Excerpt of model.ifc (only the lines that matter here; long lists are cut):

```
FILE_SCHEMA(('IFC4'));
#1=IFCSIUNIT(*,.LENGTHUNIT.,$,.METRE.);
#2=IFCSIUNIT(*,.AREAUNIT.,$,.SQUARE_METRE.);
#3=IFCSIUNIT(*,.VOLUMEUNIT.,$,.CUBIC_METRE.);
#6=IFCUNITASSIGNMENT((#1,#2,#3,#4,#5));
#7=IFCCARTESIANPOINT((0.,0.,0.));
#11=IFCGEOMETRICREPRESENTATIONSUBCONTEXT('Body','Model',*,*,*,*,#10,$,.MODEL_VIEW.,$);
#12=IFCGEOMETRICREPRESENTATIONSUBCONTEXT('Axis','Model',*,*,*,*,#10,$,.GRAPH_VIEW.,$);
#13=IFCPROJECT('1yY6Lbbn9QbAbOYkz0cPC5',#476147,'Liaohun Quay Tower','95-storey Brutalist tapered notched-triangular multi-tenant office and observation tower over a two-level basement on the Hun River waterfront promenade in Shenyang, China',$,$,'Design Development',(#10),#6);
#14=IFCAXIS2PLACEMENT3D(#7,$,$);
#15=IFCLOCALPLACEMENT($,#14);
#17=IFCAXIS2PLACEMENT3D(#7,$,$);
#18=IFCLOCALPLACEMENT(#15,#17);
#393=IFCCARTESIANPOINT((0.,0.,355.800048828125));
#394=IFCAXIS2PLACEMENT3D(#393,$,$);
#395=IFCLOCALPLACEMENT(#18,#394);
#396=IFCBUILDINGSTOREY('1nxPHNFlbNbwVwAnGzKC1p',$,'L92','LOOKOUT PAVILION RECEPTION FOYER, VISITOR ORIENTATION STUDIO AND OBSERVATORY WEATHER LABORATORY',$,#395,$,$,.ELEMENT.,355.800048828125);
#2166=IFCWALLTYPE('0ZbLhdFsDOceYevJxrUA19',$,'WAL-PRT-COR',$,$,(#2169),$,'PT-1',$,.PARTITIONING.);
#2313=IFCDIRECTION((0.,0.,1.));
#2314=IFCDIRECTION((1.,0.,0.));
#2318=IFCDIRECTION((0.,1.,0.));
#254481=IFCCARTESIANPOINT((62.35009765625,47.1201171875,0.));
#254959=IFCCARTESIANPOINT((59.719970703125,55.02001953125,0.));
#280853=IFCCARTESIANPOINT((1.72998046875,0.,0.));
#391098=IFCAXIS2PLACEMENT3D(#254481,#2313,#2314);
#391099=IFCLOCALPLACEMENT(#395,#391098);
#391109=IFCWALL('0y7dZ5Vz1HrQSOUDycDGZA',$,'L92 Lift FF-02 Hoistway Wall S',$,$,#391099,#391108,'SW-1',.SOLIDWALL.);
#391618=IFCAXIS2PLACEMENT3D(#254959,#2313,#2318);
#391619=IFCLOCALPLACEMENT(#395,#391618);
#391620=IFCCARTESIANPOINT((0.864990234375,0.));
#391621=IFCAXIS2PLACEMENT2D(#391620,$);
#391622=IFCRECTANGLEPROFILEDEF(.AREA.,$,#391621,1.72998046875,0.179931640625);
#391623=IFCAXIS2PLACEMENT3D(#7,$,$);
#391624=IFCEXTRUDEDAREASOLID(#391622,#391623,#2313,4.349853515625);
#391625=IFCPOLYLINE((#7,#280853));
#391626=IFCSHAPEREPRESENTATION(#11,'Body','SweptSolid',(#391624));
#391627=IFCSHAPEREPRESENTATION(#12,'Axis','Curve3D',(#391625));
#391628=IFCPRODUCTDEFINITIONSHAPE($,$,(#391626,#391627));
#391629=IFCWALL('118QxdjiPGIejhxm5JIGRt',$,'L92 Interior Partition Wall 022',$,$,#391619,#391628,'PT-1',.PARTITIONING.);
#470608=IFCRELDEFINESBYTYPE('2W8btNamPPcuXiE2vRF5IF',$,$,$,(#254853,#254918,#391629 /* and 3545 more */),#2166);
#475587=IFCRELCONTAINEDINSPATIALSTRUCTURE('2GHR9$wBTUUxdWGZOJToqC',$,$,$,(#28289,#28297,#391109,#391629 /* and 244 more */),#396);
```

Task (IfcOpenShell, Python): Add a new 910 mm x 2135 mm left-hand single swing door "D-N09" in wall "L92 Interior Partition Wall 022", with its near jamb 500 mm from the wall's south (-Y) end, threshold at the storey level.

```python
import numpy as np
import ifcopenshell
import ifcopenshell.api.feature
import ifcopenshell.api.geometry
import ifcopenshell.api.root
import ifcopenshell.api.spatial
import ifcopenshell.geom
import ifcopenshell.util.element
import ifcopenshell.util.placement
import ifcopenshell.util.representation
import ifcopenshell.util.shape
import ifcopenshell.util.unit

model = ifcopenshell.open("model.ifc")
unit_scale = ifcopenshell.util.unit.calculate_unit_scale(model)
settings = ifcopenshell.geom.settings()


def volume(element):
    """Net volume in cubic metres, openings subtracted."""
    shape = ifcopenshell.geom.create_shape(settings, element)
    return ifcopenshell.util.shape.get_volume(shape.geometry)


wall = model.by_id(391629)
storey = ifcopenshell.util.element.get_container(wall, ifc_class="IfcBuildingStorey")
context = ifcopenshell.util.representation.get_context(model, "Model", "Body", "MODEL_VIEW")
before = volume(wall)

width, height, from_end, sill = 0.91, 2.135, 0.5, 0.0  # metres

# The wall runs along its own X axis, and the end named is its -X end.
wall_shape = ifcopenshell.geom.create_shape(settings, wall)
x, y, z = ifcopenshell.util.shape.get_vertices(wall_shape.geometry).T
start = x.min() + from_end
face, thickness = float(y.min()), float(y.max() - y.min())
wall_matrix = ifcopenshell.util.placement.get_local_placement(wall.ObjectPlacement)
level = ifcopenshell.util.placement.get_local_placement(storey.ObjectPlacement)[2, 3]


def in_wall(x, y):
    """Placement at x, y metres in the wall's axes, at sill height."""
    matrix = wall_matrix.copy()
    matrix[:, 3] = wall_matrix @ np.array([x / unit_scale, y / unit_scale, 0.0, 1.0])
    matrix[2, 3] = level + sill / unit_scale
    return matrix


# Opening: a box that overshoots both wall faces by 50 mm.
opening = ifcopenshell.api.root.create_entity(model, ifc_class="IfcOpeningElement", predefined_type="OPENING")
box = ifcopenshell.api.geometry.add_wall_representation(
    model, context=context, length=width, height=height, thickness=thickness + 0.1
)
ifcopenshell.api.geometry.assign_representation(model, product=opening, representation=box)
ifcopenshell.api.geometry.edit_object_placement(model, product=opening, matrix=in_wall(start, face - 0.05), is_si=False)
ifcopenshell.api.feature.add_feature(model, feature=opening, element=wall)

door = ifcopenshell.api.root.create_entity(model, ifc_class="IfcDoor", name="D-N09", predefined_type="DOOR")
door.OverallWidth, door.OverallHeight = width / unit_scale, height / unit_scale
door.OperationType = "SINGLE_SWING_LEFT"
body = ifcopenshell.api.geometry.add_door_representation(
    model,
    context=context,
    overall_width=door.OverallWidth,
    overall_height=door.OverallHeight,
    operation_type="SINGLE_SWING_LEFT",
    lining_properties={"LiningDepth": thickness / unit_scale, "ThresholdDepth": thickness / unit_scale},
)
ifcopenshell.api.geometry.assign_representation(model, product=door, representation=body)
ifcopenshell.api.spatial.assign_container(model, products=[door], relating_structure=storey)
ifcopenshell.api.feature.add_filling(model, opening=opening, element=door)

# The lining spans the wall, so the door starts at the wall face.
ifcopenshell.api.geometry.edit_object_placement(model, product=door, matrix=in_wall(start, face), is_si=False)

after = volume(wall)

print(f"wall volume {before:.3f} -> {after:.3f} m3")

model.write("model_updated.ifc")
```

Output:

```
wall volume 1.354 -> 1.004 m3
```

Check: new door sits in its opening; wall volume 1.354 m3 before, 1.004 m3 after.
